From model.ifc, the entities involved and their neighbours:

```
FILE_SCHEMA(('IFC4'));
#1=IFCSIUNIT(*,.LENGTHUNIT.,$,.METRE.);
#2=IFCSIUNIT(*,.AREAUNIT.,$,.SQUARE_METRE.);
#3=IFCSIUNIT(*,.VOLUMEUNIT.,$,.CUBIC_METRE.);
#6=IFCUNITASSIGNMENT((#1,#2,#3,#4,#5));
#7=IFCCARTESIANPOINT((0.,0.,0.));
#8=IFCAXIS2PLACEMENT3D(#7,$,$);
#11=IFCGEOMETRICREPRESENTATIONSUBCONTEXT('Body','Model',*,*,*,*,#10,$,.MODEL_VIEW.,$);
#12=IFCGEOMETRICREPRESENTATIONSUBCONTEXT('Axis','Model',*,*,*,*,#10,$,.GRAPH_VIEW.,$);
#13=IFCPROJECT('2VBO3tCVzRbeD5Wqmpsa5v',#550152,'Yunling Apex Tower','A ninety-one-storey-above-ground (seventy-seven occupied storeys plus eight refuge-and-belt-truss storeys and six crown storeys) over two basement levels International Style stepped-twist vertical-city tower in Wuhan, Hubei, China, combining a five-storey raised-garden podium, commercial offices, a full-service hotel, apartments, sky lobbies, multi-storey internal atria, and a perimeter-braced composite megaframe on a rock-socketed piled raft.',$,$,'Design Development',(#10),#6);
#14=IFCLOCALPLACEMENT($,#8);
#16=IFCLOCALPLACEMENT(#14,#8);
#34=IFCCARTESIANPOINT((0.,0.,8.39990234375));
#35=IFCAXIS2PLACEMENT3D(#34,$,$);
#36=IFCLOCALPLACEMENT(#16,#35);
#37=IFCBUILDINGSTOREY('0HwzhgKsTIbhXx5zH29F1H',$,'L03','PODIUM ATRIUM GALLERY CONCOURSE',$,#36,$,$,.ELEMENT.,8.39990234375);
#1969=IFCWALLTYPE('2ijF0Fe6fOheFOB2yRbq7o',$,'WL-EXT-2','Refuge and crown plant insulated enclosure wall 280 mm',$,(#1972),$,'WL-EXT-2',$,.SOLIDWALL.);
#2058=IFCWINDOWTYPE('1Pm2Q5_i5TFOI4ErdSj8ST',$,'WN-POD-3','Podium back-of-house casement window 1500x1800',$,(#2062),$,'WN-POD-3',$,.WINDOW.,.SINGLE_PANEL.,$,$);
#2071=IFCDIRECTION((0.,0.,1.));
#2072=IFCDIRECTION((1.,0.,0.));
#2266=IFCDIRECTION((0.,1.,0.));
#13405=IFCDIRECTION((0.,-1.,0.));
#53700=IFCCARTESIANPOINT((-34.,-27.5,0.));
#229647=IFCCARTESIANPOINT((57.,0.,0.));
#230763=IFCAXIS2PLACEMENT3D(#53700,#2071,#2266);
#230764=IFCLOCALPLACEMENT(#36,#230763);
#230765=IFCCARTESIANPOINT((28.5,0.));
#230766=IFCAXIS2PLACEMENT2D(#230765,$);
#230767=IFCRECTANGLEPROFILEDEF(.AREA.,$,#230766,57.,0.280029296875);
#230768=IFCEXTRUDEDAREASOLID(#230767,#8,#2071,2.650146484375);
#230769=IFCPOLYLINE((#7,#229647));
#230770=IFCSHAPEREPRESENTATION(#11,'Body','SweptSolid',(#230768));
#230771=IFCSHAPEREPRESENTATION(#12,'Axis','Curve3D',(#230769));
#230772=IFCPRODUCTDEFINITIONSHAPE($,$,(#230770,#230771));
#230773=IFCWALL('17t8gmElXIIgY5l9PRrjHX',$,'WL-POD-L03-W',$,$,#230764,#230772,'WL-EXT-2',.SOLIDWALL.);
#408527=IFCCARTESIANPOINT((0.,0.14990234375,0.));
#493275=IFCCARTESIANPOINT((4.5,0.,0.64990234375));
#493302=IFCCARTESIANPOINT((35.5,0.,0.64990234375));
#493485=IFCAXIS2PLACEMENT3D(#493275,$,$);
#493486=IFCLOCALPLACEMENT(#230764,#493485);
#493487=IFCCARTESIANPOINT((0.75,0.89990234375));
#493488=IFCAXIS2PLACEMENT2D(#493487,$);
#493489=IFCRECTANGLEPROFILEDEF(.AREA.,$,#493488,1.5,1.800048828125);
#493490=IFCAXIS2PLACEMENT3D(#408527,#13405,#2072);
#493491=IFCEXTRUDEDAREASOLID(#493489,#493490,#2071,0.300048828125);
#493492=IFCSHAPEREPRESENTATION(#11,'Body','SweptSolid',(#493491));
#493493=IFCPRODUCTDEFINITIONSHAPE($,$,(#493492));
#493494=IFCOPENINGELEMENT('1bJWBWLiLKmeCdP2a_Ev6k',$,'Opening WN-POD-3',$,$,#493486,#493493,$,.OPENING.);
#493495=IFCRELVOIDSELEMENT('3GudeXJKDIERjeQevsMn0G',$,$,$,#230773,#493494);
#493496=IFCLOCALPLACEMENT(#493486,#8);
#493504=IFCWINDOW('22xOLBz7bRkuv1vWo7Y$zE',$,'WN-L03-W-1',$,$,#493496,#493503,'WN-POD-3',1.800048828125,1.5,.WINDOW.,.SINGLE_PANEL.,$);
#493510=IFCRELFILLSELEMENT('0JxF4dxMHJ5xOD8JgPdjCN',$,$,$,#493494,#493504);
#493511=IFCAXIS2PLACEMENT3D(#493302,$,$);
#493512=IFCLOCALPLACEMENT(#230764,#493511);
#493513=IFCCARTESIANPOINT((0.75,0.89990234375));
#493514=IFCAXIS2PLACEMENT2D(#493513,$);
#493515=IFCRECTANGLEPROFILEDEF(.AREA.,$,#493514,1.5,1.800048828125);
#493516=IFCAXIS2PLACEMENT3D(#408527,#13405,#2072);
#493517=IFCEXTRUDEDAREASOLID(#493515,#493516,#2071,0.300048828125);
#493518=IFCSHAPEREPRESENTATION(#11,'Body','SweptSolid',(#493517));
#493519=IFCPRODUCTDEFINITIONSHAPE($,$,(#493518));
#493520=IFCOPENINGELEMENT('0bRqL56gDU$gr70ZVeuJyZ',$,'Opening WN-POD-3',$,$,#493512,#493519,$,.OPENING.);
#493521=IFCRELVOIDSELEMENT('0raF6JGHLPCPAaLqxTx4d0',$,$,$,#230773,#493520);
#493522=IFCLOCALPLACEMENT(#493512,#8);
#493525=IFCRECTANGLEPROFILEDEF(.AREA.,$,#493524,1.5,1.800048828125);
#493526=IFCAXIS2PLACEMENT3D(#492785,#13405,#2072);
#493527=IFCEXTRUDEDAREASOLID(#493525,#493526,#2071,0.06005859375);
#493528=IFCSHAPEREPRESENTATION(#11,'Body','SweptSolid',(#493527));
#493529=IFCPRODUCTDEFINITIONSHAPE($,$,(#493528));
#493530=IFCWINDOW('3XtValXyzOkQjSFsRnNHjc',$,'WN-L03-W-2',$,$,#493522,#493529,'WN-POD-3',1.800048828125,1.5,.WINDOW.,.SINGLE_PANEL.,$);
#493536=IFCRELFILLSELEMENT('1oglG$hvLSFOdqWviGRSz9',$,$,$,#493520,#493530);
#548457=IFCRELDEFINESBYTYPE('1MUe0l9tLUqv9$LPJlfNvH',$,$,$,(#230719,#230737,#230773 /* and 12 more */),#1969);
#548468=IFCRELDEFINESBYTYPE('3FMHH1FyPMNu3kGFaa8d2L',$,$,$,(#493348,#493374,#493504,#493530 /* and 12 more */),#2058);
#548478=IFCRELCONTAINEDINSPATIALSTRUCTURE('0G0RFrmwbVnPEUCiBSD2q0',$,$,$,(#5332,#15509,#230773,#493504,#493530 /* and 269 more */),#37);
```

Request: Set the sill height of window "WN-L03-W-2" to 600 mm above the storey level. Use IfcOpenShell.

```python
import numpy as np
import ifcopenshell
import ifcopenshell.api.geometry
import ifcopenshell.geom
import ifcopenshell.util.element
import ifcopenshell.util.placement
import ifcopenshell.util.shape
import ifcopenshell.util.unit

model = ifcopenshell.open("model.ifc")
unit_scale = ifcopenshell.util.unit.calculate_unit_scale(model)

window = model.by_guid("3XtValXyzOkQjSFsRnNHjc")
opening = window.FillsVoids[0].RelatingOpeningElement
storey = ifcopenshell.util.element.get_container(window, ifc_class="IfcBuildingStorey")
level = ifcopenshell.util.placement.get_local_placement(storey.ObjectPlacement)[2, 3]

# The opening's origin need not be at the sill, so measure its lowest point.
shape = ifcopenshell.geom.create_shape(ifcopenshell.geom.settings(), opening)
bottom = ifcopenshell.util.shape.get_shape_bottom_elevation(shape, shape.geometry) / unit_scale
dz = level + 0.6 / unit_scale - bottom

shift = np.array([0.0, 0.0, dz])
# The window is placed relative to its opening, so it follows when the opening moves.
matrix = ifcopenshell.util.placement.get_local_placement(opening.ObjectPlacement)
matrix[:3, 3] += shift
ifcopenshell.api.geometry.edit_object_placement(
    model, product=opening, matrix=matrix, is_si=False, should_transform_children=True
)

print(f"moved by {dz * unit_scale:+.3f} m")

model.write("model-out.ifc")
```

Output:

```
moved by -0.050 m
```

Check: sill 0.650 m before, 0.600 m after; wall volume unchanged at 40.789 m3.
